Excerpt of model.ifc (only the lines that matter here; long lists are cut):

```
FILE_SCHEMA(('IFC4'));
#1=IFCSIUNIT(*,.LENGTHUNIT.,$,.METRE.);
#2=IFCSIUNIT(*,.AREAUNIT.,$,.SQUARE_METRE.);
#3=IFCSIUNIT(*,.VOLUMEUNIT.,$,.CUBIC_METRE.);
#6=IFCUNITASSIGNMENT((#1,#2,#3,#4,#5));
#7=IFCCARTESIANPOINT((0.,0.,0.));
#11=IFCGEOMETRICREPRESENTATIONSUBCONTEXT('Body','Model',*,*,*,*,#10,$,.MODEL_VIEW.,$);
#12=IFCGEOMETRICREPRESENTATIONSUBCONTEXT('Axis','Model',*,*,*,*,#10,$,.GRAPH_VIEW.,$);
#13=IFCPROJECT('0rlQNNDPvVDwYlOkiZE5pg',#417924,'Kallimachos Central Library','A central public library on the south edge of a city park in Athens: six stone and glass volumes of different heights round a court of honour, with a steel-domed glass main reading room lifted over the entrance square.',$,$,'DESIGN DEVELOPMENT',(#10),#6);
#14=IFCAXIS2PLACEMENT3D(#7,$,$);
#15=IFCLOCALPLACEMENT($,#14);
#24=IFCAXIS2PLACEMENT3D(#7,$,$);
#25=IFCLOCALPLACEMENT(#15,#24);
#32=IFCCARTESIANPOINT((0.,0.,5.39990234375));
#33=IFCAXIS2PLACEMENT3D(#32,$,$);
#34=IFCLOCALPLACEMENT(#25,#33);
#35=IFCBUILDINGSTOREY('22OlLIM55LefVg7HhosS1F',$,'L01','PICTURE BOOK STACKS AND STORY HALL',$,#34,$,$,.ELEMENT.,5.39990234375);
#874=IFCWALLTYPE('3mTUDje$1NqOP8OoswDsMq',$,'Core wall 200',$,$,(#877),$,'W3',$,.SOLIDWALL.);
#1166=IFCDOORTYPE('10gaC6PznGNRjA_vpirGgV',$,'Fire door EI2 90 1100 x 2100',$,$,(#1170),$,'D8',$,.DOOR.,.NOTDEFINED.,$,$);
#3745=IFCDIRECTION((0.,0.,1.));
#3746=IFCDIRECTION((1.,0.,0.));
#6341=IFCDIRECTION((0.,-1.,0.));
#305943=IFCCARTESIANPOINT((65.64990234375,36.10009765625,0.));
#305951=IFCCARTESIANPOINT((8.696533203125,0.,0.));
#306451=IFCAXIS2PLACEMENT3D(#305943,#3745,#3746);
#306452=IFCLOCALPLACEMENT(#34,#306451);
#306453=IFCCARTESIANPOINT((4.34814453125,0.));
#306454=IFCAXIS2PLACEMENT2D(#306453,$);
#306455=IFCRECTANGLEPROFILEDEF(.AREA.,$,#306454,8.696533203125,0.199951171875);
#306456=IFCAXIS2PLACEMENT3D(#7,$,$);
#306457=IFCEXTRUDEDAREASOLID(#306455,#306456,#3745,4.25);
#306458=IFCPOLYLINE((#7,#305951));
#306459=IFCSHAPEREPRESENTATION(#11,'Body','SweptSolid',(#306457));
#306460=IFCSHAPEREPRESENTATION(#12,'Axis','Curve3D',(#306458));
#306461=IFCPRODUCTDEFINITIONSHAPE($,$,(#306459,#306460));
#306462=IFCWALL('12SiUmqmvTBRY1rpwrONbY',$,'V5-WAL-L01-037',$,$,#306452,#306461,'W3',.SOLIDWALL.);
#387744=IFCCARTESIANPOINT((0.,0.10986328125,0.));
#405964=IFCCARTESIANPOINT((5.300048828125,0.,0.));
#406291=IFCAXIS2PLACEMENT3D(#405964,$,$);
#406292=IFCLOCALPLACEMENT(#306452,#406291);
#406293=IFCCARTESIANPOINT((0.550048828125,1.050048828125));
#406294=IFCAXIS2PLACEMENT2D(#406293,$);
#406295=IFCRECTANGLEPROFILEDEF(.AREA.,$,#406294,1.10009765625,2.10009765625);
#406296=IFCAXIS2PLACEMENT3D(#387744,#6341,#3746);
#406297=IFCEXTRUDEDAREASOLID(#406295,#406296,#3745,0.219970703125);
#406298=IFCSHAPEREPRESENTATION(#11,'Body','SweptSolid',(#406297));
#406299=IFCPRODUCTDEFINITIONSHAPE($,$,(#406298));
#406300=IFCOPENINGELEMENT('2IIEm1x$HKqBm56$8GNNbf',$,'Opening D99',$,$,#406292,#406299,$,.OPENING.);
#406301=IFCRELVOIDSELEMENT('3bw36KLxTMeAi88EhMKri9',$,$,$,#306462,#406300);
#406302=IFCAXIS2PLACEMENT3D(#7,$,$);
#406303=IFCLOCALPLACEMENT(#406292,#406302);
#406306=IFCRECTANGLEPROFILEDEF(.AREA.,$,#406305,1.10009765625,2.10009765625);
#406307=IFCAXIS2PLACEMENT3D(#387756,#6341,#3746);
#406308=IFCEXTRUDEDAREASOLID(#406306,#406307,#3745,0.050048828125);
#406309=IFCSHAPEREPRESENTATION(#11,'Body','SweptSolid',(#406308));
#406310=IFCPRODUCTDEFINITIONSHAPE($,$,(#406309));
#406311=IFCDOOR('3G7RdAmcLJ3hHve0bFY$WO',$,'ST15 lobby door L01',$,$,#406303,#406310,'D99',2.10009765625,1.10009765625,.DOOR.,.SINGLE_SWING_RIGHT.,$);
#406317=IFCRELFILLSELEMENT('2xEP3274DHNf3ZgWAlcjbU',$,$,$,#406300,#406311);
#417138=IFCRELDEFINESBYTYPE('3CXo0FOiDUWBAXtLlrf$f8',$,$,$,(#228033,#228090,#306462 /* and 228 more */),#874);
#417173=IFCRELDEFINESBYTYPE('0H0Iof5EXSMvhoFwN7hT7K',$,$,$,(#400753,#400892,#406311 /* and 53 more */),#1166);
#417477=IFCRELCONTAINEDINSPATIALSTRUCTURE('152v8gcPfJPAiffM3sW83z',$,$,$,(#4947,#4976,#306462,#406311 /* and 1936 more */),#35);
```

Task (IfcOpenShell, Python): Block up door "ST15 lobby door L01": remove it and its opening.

```python
import ifcopenshell
import ifcopenshell.api.feature
import ifcopenshell.api.root
import ifcopenshell.geom
import ifcopenshell.util.shape

model = ifcopenshell.open("model.ifc")
settings = ifcopenshell.geom.settings()


def volume(element):
    """Net volume in cubic metres, openings subtracted."""
    shape = ifcopenshell.geom.create_shape(settings, element)
    return ifcopenshell.util.shape.get_volume(shape.geometry)


door = model.by_guid("3G7RdAmcLJ3hHve0bFY$WO")
opening = door.FillsVoids[0].RelatingOpeningElement
wall = opening.VoidsElements[0].RelatingBuildingElement
before = volume(wall)

ifcopenshell.api.root.remove_product(model, product=door)
ifcopenshell.api.feature.remove_feature(model, feature=opening)

after = volume(wall)

print(f"wall volume {before:.3f} -> {after:.3f} m3")

model.write("model_v2.ifc")
```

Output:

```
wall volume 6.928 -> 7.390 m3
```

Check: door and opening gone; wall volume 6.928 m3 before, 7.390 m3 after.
